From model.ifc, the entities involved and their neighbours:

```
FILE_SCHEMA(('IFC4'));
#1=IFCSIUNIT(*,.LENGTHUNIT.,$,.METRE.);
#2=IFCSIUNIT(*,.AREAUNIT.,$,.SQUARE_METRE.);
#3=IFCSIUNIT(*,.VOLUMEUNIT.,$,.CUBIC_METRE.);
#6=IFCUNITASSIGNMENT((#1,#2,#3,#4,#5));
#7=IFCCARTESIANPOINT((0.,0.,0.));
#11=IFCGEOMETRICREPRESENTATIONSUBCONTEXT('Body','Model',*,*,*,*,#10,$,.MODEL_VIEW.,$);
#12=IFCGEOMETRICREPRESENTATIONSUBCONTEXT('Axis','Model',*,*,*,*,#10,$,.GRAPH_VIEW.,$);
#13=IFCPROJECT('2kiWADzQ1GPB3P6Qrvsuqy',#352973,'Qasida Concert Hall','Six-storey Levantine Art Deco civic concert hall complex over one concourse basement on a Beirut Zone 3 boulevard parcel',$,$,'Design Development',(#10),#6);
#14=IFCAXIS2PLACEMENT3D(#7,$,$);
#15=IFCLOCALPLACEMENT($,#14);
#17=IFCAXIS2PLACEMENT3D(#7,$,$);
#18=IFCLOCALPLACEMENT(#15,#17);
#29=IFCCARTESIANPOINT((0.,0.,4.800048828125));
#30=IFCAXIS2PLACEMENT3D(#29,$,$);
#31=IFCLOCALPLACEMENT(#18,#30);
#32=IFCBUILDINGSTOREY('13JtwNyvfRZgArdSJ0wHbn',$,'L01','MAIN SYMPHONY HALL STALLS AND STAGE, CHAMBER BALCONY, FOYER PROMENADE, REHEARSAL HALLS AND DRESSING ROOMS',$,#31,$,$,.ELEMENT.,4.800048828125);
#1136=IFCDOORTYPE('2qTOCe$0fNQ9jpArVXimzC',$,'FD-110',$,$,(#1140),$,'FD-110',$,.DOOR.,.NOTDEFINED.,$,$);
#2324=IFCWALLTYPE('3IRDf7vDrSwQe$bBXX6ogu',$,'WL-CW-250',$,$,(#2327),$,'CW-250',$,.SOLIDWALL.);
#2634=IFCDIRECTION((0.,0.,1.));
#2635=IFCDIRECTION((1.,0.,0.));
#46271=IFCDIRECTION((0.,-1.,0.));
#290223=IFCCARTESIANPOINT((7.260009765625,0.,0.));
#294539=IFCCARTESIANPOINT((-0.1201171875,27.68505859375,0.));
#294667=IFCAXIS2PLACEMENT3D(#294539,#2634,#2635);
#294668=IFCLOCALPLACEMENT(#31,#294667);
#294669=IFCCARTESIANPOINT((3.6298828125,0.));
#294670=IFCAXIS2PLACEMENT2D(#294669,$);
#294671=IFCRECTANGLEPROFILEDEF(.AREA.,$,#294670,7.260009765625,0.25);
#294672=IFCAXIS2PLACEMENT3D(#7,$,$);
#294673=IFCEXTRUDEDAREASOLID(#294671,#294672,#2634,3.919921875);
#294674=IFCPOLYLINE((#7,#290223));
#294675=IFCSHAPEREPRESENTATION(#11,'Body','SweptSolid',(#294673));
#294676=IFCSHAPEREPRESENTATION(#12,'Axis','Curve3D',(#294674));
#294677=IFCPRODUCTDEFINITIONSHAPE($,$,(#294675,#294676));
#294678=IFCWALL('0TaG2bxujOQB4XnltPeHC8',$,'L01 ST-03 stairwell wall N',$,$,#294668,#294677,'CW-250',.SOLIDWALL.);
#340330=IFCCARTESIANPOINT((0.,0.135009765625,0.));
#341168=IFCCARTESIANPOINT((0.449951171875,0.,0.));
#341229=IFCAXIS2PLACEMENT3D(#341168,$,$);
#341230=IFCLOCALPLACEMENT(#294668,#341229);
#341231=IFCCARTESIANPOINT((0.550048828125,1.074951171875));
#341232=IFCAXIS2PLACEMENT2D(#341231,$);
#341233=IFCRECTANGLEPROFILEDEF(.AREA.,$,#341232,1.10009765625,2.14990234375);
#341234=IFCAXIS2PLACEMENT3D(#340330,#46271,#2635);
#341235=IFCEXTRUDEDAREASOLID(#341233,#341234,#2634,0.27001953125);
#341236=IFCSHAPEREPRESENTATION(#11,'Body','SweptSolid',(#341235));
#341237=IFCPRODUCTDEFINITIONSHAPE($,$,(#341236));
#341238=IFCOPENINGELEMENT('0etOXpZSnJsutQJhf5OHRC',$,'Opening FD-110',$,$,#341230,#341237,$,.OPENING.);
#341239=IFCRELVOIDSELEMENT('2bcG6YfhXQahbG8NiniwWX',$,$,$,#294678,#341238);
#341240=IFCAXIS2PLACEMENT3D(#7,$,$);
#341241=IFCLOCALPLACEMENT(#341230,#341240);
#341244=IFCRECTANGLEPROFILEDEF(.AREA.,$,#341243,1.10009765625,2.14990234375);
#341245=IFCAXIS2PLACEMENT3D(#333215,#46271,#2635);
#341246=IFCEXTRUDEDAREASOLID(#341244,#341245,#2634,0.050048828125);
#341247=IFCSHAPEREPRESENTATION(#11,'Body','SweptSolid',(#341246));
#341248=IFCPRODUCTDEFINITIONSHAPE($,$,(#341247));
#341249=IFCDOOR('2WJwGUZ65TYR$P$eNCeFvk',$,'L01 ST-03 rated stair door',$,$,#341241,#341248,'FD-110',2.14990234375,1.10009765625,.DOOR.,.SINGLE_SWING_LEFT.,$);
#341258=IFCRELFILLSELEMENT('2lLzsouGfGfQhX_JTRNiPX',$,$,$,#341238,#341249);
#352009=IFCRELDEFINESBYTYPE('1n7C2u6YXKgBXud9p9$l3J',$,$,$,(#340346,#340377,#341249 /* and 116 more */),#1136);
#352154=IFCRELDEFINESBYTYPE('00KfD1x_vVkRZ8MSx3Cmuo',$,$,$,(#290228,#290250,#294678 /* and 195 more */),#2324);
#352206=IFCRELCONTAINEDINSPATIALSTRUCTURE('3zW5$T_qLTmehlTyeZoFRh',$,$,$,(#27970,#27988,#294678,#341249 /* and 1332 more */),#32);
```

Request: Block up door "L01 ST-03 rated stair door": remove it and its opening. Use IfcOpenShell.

```python
import ifcopenshell
import ifcopenshell.api.feature
import ifcopenshell.api.root
import ifcopenshell.geom
import ifcopenshell.util.shape

model = ifcopenshell.open("model.ifc")
settings = ifcopenshell.geom.settings()


def volume(element):
    """Net volume in cubic metres, openings subtracted."""
    shape = ifcopenshell.geom.create_shape(settings, element)
    return ifcopenshell.util.shape.get_volume(shape.geometry)


door = model.by_id(341249)
opening = door.FillsVoids[0].RelatingOpeningElement
wall = opening.VoidsElements[0].RelatingBuildingElement
before = volume(wall)

ifcopenshell.api.root.remove_product(model, product=door)
ifcopenshell.api.feature.remove_feature(model, feature=opening)

after = volume(wall)

print(f"wall volume {before:.3f} -> {after:.3f} m3")

model.write("model_edited.ifc")
```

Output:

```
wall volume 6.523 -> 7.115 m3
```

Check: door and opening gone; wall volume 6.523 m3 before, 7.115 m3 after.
